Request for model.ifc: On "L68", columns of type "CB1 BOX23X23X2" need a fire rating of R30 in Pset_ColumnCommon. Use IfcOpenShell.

First a look at what the model holds.

```python
import ifcopenshell
import ifcopenshell.util.element

model = ifcopenshell.open("model.ifc")
print(model.schema)
storey = next(s for s in model.by_type("IfcBuildingStorey") if s.Name == "L68")
columns = [e for e in ifcopenshell.util.element.get_decomposition(storey) if e.is_a("IfcColumn")]
seen = {}
for e in columns:
    element_type = ifcopenshell.util.element.get_type(e)
    key = (element_type.Name if element_type != e and element_type else None, ifcopenshell.util.element.get_pset(e, "Pset_ColumnCommon", "FireRating"))
    seen[key] = seen.get(key, 0) + 1
for (name, value), count in sorted(seen.items(), key=str):
    print(count, "x", name, "|", value)
```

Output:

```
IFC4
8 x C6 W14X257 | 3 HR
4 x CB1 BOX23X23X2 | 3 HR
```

```python
import ifcopenshell
import ifcopenshell.api.pset
import ifcopenshell.util.element

model = ifcopenshell.open("model.ifc")

storey = next(s for s in model.by_type("IfcBuildingStorey") if s.Name == "L68")
columns = [e for e in ifcopenshell.util.element.get_decomposition(storey) if e.is_a("IfcColumn")]

count = 0
for e in columns:
    element_type = ifcopenshell.util.element.get_type(e)
    if element_type in (None, e) or element_type.Name != "CB1 BOX23X23X2":
        continue
    found = ifcopenshell.util.element.get_pset(e, "Pset_ColumnCommon", should_inherit=False)
    if found:
        pset = model.by_id(found["id"])
        if len(ifcopenshell.util.element.get_elements_by_pset(pset)) > 1:
            pset = ifcopenshell.api.pset.unshare_pset(model, products=[e], pset=pset)[0]
    else:
        pset = ifcopenshell.api.pset.add_pset(model, product=e, name="Pset_ColumnCommon")
    ifcopenshell.api.pset.edit_pset(model, pset=pset, properties={"FireRating": "R30"})
    count += 1

print(count, "columns updated")

model.write("model_rev.ifc")
```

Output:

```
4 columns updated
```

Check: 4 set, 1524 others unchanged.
